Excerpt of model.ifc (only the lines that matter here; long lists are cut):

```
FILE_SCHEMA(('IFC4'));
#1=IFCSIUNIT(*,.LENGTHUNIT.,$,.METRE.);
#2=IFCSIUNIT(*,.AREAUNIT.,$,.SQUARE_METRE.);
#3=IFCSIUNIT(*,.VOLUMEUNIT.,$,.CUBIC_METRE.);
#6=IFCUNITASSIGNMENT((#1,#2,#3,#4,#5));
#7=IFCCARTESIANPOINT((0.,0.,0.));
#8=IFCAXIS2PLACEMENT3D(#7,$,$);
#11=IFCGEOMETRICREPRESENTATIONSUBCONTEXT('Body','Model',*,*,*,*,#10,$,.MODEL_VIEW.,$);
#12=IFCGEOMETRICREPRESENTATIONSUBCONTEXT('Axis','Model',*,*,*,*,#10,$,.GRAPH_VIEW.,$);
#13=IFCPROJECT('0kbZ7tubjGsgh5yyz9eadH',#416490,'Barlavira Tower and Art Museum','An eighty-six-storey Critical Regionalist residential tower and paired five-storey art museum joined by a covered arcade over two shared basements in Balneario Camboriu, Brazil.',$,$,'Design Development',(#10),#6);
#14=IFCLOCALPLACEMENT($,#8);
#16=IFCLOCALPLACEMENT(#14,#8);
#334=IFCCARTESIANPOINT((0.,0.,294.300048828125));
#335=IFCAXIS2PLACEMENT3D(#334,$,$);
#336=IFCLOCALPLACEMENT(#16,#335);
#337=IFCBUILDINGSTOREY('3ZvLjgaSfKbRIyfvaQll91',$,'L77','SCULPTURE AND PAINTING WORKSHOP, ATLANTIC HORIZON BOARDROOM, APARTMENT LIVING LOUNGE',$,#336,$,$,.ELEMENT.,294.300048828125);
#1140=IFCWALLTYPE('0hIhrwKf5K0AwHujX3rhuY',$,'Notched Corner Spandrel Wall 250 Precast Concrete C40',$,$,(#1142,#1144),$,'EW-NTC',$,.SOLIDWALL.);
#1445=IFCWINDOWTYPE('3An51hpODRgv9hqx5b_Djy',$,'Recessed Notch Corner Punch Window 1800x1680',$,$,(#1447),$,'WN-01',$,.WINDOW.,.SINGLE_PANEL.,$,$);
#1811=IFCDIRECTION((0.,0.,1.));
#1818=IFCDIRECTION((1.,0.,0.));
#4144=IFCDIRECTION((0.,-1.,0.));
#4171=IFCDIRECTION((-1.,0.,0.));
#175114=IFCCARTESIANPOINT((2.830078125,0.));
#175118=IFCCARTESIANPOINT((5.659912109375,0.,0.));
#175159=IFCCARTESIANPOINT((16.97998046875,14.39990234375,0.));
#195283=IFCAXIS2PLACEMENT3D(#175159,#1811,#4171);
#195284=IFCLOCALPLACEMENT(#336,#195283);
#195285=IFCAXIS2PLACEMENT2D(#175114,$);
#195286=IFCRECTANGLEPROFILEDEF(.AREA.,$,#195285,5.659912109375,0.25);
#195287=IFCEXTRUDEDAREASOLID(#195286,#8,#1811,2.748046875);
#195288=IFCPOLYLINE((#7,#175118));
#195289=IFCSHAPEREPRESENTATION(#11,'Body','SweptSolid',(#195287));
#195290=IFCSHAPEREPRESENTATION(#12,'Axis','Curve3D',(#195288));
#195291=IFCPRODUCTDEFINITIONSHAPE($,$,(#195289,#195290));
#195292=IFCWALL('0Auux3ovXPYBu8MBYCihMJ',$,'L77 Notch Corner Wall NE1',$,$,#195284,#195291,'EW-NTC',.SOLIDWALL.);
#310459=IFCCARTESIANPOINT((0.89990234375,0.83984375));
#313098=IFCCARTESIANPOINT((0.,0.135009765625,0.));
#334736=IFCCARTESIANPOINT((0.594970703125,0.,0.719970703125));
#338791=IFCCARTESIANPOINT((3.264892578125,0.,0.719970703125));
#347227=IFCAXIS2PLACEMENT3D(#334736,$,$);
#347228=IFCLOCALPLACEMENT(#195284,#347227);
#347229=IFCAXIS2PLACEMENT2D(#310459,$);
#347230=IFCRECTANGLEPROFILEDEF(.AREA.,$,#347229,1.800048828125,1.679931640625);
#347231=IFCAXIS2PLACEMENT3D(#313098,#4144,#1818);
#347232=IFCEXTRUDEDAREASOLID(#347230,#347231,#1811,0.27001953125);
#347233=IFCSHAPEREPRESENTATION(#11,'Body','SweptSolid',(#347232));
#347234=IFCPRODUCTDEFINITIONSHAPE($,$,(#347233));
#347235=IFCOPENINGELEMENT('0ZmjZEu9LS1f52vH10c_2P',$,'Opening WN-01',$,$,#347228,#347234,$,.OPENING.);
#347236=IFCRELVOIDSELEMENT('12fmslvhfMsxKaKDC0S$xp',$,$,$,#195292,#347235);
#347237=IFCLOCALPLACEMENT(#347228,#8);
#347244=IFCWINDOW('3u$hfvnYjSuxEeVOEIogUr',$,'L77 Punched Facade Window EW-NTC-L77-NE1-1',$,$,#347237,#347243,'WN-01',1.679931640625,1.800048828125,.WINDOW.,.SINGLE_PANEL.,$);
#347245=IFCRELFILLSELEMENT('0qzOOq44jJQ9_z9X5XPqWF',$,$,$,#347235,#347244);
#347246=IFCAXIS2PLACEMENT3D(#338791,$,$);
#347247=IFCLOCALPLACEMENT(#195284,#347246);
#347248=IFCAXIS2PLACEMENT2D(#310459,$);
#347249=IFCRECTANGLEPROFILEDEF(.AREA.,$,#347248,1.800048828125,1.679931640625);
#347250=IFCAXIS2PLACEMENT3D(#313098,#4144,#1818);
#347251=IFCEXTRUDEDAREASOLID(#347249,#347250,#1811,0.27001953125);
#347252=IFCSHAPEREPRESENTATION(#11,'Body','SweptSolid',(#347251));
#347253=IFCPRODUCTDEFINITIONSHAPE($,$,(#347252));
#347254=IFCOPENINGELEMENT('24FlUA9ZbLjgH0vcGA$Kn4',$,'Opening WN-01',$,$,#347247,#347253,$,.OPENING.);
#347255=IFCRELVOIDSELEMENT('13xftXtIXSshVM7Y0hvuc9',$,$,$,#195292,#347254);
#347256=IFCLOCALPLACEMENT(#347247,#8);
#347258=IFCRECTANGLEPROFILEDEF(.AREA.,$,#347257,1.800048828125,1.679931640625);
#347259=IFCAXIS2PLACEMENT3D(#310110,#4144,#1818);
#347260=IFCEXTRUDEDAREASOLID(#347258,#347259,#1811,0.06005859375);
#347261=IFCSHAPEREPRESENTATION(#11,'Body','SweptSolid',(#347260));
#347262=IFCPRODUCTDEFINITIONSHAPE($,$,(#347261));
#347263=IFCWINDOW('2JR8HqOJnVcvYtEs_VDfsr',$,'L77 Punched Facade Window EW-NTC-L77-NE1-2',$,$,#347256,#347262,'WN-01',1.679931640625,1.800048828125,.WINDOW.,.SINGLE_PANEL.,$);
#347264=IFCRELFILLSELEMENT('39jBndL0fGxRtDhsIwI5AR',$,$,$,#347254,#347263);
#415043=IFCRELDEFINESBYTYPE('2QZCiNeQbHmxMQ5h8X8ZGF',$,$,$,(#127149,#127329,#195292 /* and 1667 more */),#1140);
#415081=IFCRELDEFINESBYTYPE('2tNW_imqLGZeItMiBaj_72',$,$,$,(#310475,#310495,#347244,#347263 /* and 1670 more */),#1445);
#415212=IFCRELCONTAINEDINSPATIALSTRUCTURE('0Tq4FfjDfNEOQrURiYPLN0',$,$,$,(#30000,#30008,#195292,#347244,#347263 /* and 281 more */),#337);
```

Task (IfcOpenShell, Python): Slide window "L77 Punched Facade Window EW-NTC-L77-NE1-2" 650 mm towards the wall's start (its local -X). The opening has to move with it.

```python
import ifcopenshell
import ifcopenshell.api.geometry
import ifcopenshell.util.placement

model = ifcopenshell.open("model.ifc")

window = model.by_guid("2JR8HqOJnVcvYtEs_VDfsr")
opening = window.FillsVoids[0].RelatingOpeningElement
wall = opening.VoidsElements[0].RelatingBuildingElement

wall_matrix = ifcopenshell.util.placement.get_local_placement(wall.ObjectPlacement)
shift = wall_matrix[:3, 0] * -0.65
before = ifcopenshell.util.placement.get_local_placement(window.ObjectPlacement)[:3, 3].copy()

# The window is placed relative to its opening, so it follows when the opening moves.
matrix = ifcopenshell.util.placement.get_local_placement(opening.ObjectPlacement)
matrix[:3, 3] += shift
ifcopenshell.api.geometry.edit_object_placement(
    model, product=opening, matrix=matrix, is_si=False, should_transform_children=True
)

after = ifcopenshell.util.placement.get_local_placement(window.ObjectPlacement)[:3, 3]
print("window moved by", (after - before).round(3) + 0.0)

model.write("model-out.ifc")
```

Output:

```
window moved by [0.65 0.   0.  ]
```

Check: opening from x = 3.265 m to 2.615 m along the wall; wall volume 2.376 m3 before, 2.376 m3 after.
